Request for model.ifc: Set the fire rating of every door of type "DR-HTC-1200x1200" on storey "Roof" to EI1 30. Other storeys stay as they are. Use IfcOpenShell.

First a look at what the model holds.

```python
import ifcopenshell
import ifcopenshell.util.element

model = ifcopenshell.open("model.ifc")
print(model.schema)
storey = next(s for s in model.by_type("IfcBuildingStorey") if s.Name == "Roof")
doors = [e for e in ifcopenshell.util.element.get_decomposition(storey) if e.is_a("IfcDoor")]
seen = {}
for e in doors:
    element_type = ifcopenshell.util.element.get_type(e)
    key = (element_type.Name if element_type != e and element_type else None, ifcopenshell.util.element.get_pset(e, "Pset_DoorCommon", "FireRating"))
    seen[key] = seen.get(key, 0) + 1
for (name, value), count in sorted(seen.items(), key=str):
    print(count, "x", name, "|", value)
```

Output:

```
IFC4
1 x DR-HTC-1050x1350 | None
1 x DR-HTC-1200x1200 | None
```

```python
import ifcopenshell
import ifcopenshell.api.pset
import ifcopenshell.util.element

model = ifcopenshell.open("model.ifc")

storey = next(s for s in model.by_type("IfcBuildingStorey") if s.Name == "Roof")
doors = [e for e in ifcopenshell.util.element.get_decomposition(storey) if e.is_a("IfcDoor")]

count = 0
for e in doors:
    element_type = ifcopenshell.util.element.get_type(e)
    if element_type in (None, e) or element_type.Name != "DR-HTC-1200x1200":
        continue
    # add_pset returns the element's existing set when there is one.
    pset = ifcopenshell.api.pset.add_pset(model, product=e, name="Pset_DoorCommon")
    ifcopenshell.api.pset.edit_pset(model, pset=pset, properties={"FireRating": "EI1 30"})
    count += 1

print(count, "doors updated")

model.write("model-out.ifc")
```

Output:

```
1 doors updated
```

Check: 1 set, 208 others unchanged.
